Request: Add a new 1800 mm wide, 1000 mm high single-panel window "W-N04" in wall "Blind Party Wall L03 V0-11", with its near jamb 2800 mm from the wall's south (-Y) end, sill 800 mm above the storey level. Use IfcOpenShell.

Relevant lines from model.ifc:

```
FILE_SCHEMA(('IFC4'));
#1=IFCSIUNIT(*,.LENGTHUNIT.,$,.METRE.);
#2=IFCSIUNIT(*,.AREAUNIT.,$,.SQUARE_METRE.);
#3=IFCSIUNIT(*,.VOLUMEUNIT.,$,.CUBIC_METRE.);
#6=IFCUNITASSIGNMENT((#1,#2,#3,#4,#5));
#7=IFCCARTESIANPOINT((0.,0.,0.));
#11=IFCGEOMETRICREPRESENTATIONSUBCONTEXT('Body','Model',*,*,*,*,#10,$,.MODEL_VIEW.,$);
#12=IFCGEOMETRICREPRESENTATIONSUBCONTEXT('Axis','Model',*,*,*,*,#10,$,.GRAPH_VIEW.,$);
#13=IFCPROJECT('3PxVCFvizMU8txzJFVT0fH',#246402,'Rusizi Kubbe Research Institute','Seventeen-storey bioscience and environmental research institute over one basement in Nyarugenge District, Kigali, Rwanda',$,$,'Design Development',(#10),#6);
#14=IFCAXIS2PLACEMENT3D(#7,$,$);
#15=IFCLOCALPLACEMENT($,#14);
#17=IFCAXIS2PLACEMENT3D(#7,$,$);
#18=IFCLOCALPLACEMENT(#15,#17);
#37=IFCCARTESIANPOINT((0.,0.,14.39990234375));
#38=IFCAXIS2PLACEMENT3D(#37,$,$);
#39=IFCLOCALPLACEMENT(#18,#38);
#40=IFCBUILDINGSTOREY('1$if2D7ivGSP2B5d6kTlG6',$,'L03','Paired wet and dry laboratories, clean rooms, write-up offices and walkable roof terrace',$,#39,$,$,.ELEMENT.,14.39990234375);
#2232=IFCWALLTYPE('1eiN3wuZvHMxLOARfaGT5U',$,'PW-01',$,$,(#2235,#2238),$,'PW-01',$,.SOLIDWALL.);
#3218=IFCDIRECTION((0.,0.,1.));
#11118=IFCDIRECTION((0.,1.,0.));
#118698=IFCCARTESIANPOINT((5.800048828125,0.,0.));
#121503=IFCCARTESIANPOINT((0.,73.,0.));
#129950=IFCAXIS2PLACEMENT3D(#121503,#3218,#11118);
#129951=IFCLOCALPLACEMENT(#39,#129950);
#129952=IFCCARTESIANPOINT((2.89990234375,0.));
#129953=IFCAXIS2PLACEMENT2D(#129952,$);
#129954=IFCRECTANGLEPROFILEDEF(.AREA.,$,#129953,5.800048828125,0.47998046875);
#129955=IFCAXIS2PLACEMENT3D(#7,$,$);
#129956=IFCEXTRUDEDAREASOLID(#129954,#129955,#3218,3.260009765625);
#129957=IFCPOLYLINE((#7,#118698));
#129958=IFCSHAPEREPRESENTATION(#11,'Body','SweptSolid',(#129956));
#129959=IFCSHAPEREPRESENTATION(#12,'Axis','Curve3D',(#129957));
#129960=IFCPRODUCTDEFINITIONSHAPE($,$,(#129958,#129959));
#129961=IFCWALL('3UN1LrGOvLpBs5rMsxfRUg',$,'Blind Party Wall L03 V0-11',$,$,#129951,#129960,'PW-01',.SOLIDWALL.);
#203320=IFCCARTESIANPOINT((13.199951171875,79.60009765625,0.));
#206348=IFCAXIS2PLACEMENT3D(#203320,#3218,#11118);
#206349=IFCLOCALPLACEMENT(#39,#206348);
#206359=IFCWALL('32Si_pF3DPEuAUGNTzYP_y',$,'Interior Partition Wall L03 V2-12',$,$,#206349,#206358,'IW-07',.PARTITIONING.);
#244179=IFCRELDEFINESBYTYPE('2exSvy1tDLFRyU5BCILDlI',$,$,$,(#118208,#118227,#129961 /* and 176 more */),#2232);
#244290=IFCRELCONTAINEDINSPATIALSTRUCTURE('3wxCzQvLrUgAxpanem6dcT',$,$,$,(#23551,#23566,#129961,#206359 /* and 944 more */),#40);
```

```python
import numpy as np
import ifcopenshell
import ifcopenshell.api.feature
import ifcopenshell.api.geometry
import ifcopenshell.api.root
import ifcopenshell.api.spatial
import ifcopenshell.geom
import ifcopenshell.util.element
import ifcopenshell.util.placement
import ifcopenshell.util.representation
import ifcopenshell.util.shape
import ifcopenshell.util.unit

model = ifcopenshell.open("model.ifc")
unit_scale = ifcopenshell.util.unit.calculate_unit_scale(model)
settings = ifcopenshell.geom.settings()


def volume(element):
    """Net volume in cubic metres, openings subtracted."""
    shape = ifcopenshell.geom.create_shape(settings, element)
    return ifcopenshell.util.shape.get_volume(shape.geometry)


wall = model.by_guid("3UN1LrGOvLpBs5rMsxfRUg")
storey = ifcopenshell.util.element.get_container(wall, ifc_class="IfcBuildingStorey")
context = ifcopenshell.util.representation.get_context(model, "Model", "Body", "MODEL_VIEW")
before = volume(wall)

width, height, from_end, sill = 1.8, 1, 2.8, 0.8  # metres

# The wall runs along its own X axis, and the end named is its -X end.
wall_shape = ifcopenshell.geom.create_shape(settings, wall)
x, y, z = ifcopenshell.util.shape.get_vertices(wall_shape.geometry).T
start = x.min() + from_end
face, thickness = float(y.min()), float(y.max() - y.min())
wall_matrix = ifcopenshell.util.placement.get_local_placement(wall.ObjectPlacement)
level = ifcopenshell.util.placement.get_local_placement(storey.ObjectPlacement)[2, 3]


def in_wall(x, y):
    """Placement at x, y metres in the wall's axes, at sill height."""
    matrix = wall_matrix.copy()
    matrix[:, 3] = wall_matrix @ np.array([x / unit_scale, y / unit_scale, 0.0, 1.0])
    matrix[2, 3] = level + sill / unit_scale
    return matrix


# Opening: a box that overshoots both wall faces by 50 mm.
opening = ifcopenshell.api.root.create_entity(model, ifc_class="IfcOpeningElement", predefined_type="OPENING")
box = ifcopenshell.api.geometry.add_wall_representation(
    model, context=context, length=width, height=height, thickness=thickness + 0.1
)
ifcopenshell.api.geometry.assign_representation(model, product=opening, representation=box)
ifcopenshell.api.geometry.edit_object_placement(model, product=opening, matrix=in_wall(start, face - 0.05), is_si=False)
ifcopenshell.api.feature.add_feature(model, feature=opening, element=wall)

window = ifcopenshell.api.root.create_entity(model, ifc_class="IfcWindow", name="W-N04", predefined_type="WINDOW")
window.OverallWidth, window.OverallHeight = width / unit_scale, height / unit_scale
window.PartitioningType = "SINGLE_PANEL"
body = ifcopenshell.api.geometry.add_window_representation(
    model,
    context=context,
    overall_width=window.OverallWidth,
    overall_height=window.OverallHeight,
    partition_type="SINGLE_PANEL",
)
ifcopenshell.api.geometry.assign_representation(model, product=window, representation=body)
ifcopenshell.api.spatial.assign_container(model, products=[window], relating_structure=storey)
ifcopenshell.api.feature.add_filling(model, opening=opening, element=window)

# Centre the window in the wall's thickness.
ifcopenshell.api.geometry.edit_object_placement(model, product=window, matrix=in_wall(start, face), is_si=False)
window_shape = ifcopenshell.geom.create_shape(settings, window)
depth = ifcopenshell.util.shape.get_vertices(window_shape.geometry)[:, 1]
offset = face + thickness / 2 - (depth.min() + depth.max()) / 2
ifcopenshell.api.geometry.edit_object_placement(model, product=window, matrix=in_wall(start, offset), is_si=False)

after = volume(wall)

print(f"wall volume {before:.3f} -> {after:.3f} m3")

model.write("model_rev.ifc")
```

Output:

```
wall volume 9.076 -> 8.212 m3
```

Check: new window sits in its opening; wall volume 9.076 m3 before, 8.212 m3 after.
